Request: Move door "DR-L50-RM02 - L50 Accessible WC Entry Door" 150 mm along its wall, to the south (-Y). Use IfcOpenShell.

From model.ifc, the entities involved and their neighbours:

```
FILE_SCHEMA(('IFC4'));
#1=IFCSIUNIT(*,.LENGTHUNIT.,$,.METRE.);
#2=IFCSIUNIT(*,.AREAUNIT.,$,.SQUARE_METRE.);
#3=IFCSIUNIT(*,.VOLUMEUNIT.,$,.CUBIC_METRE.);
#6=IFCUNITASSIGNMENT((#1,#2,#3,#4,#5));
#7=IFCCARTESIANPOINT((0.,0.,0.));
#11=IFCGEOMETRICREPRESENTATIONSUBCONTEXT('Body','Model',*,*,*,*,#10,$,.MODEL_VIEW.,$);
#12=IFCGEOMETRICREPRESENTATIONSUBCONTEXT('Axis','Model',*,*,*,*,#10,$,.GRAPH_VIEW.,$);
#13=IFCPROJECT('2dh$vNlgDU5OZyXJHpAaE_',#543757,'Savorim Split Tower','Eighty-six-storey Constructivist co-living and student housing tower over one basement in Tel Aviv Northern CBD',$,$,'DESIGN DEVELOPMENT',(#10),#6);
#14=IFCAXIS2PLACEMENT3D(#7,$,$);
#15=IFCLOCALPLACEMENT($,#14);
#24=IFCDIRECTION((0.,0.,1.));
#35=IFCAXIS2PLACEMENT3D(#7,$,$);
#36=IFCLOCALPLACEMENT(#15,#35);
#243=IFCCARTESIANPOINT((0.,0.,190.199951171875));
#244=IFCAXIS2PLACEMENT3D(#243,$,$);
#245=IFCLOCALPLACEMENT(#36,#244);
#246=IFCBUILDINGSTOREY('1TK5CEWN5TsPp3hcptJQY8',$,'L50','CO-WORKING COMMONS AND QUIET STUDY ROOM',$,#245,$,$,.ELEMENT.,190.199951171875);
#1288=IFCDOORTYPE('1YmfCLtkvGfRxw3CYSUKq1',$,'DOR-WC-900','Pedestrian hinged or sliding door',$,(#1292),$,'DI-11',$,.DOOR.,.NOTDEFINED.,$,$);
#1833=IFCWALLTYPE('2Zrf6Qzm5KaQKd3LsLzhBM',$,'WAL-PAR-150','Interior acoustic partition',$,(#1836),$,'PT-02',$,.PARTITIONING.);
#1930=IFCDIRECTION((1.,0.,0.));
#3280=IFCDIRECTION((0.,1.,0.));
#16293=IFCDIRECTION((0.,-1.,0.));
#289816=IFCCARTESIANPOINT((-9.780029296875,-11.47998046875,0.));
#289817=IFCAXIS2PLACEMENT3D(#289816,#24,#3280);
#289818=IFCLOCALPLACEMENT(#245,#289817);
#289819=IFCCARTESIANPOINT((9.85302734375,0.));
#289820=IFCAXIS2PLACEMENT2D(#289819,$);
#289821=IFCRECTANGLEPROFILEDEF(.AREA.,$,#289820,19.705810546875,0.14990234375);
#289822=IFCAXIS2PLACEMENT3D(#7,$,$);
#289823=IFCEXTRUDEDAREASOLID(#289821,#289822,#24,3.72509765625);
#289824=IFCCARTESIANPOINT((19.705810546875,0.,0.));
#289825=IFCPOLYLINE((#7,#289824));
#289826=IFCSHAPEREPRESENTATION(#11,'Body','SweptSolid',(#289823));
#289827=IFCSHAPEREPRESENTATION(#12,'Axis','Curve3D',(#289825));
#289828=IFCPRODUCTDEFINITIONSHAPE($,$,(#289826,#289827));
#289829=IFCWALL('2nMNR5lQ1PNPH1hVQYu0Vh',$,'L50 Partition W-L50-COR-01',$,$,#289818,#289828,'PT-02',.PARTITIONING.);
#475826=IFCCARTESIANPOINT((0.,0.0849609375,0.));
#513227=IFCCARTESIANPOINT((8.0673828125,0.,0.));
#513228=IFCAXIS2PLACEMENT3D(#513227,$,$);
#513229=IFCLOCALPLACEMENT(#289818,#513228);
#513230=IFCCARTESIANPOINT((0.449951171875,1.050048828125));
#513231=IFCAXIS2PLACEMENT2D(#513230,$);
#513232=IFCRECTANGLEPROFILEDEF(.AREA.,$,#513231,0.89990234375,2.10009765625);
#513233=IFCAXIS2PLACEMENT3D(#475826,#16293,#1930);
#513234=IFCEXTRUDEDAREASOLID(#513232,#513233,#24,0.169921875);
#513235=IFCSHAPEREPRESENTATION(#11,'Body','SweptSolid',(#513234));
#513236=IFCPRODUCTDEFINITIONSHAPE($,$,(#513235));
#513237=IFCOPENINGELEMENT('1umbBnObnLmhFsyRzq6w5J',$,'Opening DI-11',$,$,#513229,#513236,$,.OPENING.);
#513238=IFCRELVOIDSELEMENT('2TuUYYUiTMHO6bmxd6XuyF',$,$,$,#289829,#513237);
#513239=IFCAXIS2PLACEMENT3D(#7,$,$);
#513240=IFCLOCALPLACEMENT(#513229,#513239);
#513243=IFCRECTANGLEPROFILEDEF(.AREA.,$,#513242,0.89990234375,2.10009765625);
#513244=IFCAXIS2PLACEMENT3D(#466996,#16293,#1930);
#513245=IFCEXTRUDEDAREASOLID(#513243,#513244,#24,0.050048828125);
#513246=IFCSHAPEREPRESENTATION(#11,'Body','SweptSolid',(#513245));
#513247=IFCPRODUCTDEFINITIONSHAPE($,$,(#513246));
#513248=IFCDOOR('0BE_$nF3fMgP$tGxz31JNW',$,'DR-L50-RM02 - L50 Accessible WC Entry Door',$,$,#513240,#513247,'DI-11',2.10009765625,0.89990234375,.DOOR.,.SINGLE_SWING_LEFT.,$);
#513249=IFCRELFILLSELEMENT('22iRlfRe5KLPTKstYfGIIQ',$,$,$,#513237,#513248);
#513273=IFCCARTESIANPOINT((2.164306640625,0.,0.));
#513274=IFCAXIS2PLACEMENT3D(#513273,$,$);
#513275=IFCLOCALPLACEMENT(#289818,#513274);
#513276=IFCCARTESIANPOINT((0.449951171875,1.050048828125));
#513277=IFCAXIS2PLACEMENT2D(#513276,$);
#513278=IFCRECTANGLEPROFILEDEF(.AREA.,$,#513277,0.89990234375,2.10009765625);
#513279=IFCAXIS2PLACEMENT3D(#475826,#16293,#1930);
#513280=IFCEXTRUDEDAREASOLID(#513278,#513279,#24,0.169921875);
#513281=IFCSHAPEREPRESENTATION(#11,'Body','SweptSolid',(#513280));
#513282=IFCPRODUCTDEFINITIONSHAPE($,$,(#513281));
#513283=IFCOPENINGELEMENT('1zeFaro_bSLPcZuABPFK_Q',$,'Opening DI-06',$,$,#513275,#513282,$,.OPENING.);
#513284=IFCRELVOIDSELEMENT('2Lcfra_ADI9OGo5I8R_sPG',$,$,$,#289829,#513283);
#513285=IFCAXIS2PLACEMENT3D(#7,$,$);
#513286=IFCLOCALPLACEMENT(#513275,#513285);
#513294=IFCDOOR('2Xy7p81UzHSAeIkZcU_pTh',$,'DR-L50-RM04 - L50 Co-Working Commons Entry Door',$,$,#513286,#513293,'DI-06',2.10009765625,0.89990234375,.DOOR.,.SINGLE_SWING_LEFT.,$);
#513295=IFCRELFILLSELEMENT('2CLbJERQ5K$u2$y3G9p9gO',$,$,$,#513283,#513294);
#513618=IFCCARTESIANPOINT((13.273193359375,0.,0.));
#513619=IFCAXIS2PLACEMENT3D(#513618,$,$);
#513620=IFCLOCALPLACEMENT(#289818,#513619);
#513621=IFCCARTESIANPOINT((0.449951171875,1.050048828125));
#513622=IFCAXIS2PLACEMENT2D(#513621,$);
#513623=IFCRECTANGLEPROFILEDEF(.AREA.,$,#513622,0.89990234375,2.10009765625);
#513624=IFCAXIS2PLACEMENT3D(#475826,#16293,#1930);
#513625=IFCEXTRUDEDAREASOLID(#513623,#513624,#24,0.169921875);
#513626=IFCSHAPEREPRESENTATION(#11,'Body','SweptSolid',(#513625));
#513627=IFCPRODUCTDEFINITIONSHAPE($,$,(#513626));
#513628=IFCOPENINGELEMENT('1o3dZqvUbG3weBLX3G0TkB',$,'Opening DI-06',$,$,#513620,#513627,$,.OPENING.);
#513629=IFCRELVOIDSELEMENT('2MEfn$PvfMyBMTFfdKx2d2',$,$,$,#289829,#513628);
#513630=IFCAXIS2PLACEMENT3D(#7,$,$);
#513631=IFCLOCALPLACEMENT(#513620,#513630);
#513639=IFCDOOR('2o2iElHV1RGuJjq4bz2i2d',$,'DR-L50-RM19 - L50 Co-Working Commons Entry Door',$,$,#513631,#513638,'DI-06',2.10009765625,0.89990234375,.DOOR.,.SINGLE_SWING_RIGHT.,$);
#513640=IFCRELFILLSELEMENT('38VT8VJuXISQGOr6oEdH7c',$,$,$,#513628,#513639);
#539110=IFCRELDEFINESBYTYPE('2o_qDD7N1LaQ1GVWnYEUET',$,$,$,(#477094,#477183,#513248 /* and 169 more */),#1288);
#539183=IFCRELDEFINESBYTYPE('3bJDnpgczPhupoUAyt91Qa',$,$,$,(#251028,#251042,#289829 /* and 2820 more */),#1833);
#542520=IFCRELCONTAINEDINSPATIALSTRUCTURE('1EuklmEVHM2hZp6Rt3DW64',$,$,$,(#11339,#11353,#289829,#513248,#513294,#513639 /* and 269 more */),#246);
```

```python
import ifcopenshell
import ifcopenshell.api.geometry
import ifcopenshell.util.placement

model = ifcopenshell.open("model.ifc")

door = model.by_guid("0BE_$nF3fMgP$tGxz31JNW")
opening = door.FillsVoids[0].RelatingOpeningElement
wall = opening.VoidsElements[0].RelatingBuildingElement

wall_matrix = ifcopenshell.util.placement.get_local_placement(wall.ObjectPlacement)
shift = wall_matrix[:3, 0] * -0.15
before = ifcopenshell.util.placement.get_local_placement(door.ObjectPlacement)[:3, 3].copy()

# The door is placed relative to its opening, so it follows when the opening moves.
matrix = ifcopenshell.util.placement.get_local_placement(opening.ObjectPlacement)
matrix[:3, 3] += shift
ifcopenshell.api.geometry.edit_object_placement(
    model, product=opening, matrix=matrix, is_si=False, should_transform_children=True
)

after = ifcopenshell.util.placement.get_local_placement(door.ObjectPlacement)[:3, 3]
print("door moved by", (after - before).round(3) + 0.0)

model.write("model_v2.ifc")
```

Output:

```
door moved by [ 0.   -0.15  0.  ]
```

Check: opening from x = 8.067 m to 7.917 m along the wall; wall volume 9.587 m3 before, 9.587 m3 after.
